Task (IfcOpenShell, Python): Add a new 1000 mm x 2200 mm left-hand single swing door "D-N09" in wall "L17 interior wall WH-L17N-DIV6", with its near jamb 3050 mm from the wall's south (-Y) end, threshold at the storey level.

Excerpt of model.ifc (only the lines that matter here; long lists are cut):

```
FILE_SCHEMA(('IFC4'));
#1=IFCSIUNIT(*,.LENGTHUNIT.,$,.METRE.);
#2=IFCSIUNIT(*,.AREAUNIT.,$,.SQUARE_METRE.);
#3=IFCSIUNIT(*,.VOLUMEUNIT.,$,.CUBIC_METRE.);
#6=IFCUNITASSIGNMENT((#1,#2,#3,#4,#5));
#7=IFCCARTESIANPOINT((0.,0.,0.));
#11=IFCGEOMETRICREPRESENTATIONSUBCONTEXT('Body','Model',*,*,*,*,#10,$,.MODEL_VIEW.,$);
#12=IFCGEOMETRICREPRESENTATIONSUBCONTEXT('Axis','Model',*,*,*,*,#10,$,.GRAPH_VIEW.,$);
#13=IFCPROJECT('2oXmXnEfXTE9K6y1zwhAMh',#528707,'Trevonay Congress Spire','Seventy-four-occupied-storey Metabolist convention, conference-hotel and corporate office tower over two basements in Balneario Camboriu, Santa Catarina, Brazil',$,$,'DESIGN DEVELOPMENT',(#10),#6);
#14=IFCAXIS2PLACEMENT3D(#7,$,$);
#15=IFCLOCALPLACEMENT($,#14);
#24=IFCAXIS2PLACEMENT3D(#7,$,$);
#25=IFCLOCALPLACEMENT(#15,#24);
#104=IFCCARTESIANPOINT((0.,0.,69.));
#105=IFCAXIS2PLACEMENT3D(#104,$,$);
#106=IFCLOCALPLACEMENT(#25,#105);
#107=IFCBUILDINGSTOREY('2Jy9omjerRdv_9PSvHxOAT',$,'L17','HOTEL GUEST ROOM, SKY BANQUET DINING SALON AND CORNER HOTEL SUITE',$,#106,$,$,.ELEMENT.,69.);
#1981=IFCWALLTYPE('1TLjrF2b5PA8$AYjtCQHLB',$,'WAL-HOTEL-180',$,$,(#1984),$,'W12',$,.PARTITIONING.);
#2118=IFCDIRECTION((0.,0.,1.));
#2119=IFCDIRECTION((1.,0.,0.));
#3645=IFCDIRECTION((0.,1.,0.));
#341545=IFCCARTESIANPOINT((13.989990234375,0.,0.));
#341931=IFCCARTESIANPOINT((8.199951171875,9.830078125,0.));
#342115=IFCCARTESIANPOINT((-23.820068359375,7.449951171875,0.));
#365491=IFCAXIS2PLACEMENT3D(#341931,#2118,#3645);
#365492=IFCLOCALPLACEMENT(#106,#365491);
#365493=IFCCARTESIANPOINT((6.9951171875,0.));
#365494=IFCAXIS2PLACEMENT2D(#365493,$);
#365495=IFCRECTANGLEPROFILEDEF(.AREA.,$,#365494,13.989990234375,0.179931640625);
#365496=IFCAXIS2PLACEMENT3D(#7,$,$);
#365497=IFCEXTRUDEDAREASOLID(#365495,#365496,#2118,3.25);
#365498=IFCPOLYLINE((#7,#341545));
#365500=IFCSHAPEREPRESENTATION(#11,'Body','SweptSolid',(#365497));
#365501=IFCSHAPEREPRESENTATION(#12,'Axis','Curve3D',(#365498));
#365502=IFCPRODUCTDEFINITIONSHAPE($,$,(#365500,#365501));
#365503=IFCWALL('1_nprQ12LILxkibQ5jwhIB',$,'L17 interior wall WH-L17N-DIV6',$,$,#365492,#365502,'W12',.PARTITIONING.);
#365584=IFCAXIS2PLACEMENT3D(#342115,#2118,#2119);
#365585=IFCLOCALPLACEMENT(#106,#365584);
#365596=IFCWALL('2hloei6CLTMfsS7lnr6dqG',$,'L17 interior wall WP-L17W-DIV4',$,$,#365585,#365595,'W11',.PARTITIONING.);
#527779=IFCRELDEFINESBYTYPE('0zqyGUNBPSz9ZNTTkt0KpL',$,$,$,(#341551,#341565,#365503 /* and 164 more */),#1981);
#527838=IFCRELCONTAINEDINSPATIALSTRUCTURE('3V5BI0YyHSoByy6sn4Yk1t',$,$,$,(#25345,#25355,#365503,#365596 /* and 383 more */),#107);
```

```python
import numpy as np
import ifcopenshell
import ifcopenshell.api.feature
import ifcopenshell.api.geometry
import ifcopenshell.api.root
import ifcopenshell.api.spatial
import ifcopenshell.geom
import ifcopenshell.util.element
import ifcopenshell.util.placement
import ifcopenshell.util.representation
import ifcopenshell.util.shape
import ifcopenshell.util.unit

model = ifcopenshell.open("model.ifc")
unit_scale = ifcopenshell.util.unit.calculate_unit_scale(model)
settings = ifcopenshell.geom.settings()


def volume(element):
    """Net volume in cubic metres, openings subtracted."""
    shape = ifcopenshell.geom.create_shape(settings, element)
    return ifcopenshell.util.shape.get_volume(shape.geometry)


wall = model.by_guid("1_nprQ12LILxkibQ5jwhIB")
storey = ifcopenshell.util.element.get_container(wall, ifc_class="IfcBuildingStorey")
context = ifcopenshell.util.representation.get_context(model, "Model", "Body", "MODEL_VIEW")
before = volume(wall)

width, height, from_end, sill = 1, 2.2, 3.05, 0.0  # metres

# The wall runs along its own X axis, and the end named is its -X end.
wall_shape = ifcopenshell.geom.create_shape(settings, wall)
x, y, z = ifcopenshell.util.shape.get_vertices(wall_shape.geometry).T
start = x.min() + from_end
face, thickness = float(y.min()), float(y.max() - y.min())
wall_matrix = ifcopenshell.util.placement.get_local_placement(wall.ObjectPlacement)
level = ifcopenshell.util.placement.get_local_placement(storey.ObjectPlacement)[2, 3]


def in_wall(x, y):
    """Placement at x, y metres in the wall's axes, at sill height."""
    matrix = wall_matrix.copy()
    matrix[:, 3] = wall_matrix @ np.array([x / unit_scale, y / unit_scale, 0.0, 1.0])
    matrix[2, 3] = level + sill / unit_scale
    return matrix


# Opening: a box that overshoots both wall faces by 50 mm.
opening = ifcopenshell.api.root.create_entity(model, ifc_class="IfcOpeningElement", predefined_type="OPENING")
box = ifcopenshell.api.geometry.add_wall_representation(
    model, context=context, length=width, height=height, thickness=thickness + 0.1
)
ifcopenshell.api.geometry.assign_representation(model, product=opening, representation=box)
ifcopenshell.api.geometry.edit_object_placement(model, product=opening, matrix=in_wall(start, face - 0.05), is_si=False)
ifcopenshell.api.feature.add_feature(model, feature=opening, element=wall)

door = ifcopenshell.api.root.create_entity(model, ifc_class="IfcDoor", name="D-N09", predefined_type="DOOR")
door.OverallWidth, door.OverallHeight = width / unit_scale, height / unit_scale
door.OperationType = "SINGLE_SWING_LEFT"
body = ifcopenshell.api.geometry.add_door_representation(
    model,
    context=context,
    overall_width=door.OverallWidth,
    overall_height=door.OverallHeight,
    operation_type="SINGLE_SWING_LEFT",
    lining_properties={"LiningDepth": thickness / unit_scale, "ThresholdDepth": thickness / unit_scale},
)
ifcopenshell.api.geometry.assign_representation(model, product=door, representation=body)
ifcopenshell.api.spatial.assign_container(model, products=[door], relating_structure=storey)
ifcopenshell.api.feature.add_filling(model, opening=opening, element=door)

# The lining spans the wall, so the door starts at the wall face.
ifcopenshell.api.geometry.edit_object_placement(model, product=door, matrix=in_wall(start, face), is_si=False)

after = volume(wall)

print(f"wall volume {before:.3f} -> {after:.3f} m3")

model.write("model-out.ifc")
```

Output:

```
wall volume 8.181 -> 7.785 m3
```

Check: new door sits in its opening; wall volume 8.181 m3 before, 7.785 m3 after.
